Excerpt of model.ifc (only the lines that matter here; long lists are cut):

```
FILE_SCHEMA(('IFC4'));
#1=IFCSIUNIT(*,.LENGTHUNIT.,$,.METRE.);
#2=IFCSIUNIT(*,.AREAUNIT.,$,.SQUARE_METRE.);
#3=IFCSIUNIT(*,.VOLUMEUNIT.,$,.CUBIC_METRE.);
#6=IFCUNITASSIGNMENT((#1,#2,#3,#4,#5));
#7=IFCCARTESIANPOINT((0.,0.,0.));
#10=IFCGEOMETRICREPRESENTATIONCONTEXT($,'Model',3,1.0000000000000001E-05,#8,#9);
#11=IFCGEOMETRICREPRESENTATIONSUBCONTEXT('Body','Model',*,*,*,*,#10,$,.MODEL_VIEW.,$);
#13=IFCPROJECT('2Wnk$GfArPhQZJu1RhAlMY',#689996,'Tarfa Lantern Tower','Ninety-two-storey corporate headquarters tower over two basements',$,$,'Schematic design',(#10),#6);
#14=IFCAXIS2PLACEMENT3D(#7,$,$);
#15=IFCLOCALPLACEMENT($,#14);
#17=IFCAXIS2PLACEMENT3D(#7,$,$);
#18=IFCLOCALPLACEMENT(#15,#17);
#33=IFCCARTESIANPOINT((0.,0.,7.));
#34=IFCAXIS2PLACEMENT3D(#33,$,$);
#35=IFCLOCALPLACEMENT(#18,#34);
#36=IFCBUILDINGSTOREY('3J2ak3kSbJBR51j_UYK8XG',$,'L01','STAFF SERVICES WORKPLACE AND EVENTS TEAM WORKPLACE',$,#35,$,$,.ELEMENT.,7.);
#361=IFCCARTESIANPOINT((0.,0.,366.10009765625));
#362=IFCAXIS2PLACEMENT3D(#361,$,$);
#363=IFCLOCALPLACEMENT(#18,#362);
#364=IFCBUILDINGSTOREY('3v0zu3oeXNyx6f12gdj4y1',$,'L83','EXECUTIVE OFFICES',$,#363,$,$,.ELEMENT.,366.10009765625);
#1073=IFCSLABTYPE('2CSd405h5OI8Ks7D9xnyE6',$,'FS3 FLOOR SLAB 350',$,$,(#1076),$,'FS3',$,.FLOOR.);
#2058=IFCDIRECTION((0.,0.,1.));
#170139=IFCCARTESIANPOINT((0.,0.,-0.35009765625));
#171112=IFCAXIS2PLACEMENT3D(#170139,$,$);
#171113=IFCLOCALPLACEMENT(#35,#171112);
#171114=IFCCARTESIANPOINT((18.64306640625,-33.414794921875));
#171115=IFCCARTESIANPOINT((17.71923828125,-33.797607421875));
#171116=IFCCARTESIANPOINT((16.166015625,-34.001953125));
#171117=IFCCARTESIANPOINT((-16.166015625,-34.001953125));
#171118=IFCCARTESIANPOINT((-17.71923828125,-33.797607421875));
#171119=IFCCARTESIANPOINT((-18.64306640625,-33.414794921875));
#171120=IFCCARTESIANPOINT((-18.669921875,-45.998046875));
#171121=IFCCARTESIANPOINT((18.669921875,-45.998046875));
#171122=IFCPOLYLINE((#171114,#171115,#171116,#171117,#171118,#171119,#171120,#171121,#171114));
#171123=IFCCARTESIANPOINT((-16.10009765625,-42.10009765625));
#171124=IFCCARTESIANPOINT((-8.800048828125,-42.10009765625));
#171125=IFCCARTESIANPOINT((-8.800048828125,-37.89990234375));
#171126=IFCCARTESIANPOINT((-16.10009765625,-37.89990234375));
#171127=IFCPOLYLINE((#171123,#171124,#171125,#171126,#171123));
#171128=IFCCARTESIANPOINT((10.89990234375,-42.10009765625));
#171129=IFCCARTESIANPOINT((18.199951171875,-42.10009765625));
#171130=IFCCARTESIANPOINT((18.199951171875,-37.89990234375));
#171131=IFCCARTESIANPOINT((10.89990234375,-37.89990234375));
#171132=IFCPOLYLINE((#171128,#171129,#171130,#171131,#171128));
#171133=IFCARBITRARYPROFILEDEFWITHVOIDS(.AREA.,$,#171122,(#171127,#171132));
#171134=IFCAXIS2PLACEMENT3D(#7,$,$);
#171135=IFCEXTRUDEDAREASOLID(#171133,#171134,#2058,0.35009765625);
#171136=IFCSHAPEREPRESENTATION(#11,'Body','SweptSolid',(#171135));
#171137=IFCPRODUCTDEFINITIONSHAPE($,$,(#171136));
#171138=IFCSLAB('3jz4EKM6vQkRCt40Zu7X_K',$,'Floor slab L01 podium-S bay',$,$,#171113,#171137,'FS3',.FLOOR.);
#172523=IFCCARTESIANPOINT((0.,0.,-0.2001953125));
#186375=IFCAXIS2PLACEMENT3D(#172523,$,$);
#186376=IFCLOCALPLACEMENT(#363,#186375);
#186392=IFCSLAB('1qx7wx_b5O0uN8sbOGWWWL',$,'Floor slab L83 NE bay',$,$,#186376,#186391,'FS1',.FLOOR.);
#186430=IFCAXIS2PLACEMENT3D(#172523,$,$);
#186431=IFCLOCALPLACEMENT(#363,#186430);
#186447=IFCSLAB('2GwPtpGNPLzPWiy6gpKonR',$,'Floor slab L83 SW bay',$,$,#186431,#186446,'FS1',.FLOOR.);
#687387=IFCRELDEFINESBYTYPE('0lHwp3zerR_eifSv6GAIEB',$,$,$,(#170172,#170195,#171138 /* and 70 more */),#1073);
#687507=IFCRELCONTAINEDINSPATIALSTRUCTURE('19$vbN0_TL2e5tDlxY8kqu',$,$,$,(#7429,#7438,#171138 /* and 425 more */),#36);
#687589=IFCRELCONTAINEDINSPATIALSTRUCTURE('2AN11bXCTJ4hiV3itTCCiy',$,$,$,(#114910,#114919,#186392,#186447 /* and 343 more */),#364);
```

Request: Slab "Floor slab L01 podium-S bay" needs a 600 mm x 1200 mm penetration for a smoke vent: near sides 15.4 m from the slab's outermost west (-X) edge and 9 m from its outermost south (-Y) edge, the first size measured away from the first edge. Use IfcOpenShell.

```python
import numpy as np
import ifcopenshell
import ifcopenshell.api.feature
import ifcopenshell.api.geometry
import ifcopenshell.api.root
import ifcopenshell.geom
import ifcopenshell.util.placement
import ifcopenshell.util.representation
import ifcopenshell.util.shape
import ifcopenshell.util.unit

model = ifcopenshell.open("model.ifc")
unit_scale = ifcopenshell.util.unit.calculate_unit_scale(model)
settings = ifcopenshell.geom.settings()


def volume(element):
    """Net volume in cubic metres, openings subtracted."""
    shape = ifcopenshell.geom.create_shape(settings, element)
    return ifcopenshell.util.shape.get_volume(shape.geometry)


slab = model.by_guid("3jz4EKM6vQkRCt40Zu7X_K")
before = volume(slab)

# Extent in the slab's own axes, in metres. The edges named are its -X and -Y sides.
slab_shape = ifcopenshell.geom.create_shape(settings, slab)
vertices = ifcopenshell.util.shape.get_vertices(slab_shape.geometry)
x_min, y_min, bottom = vertices.min(axis=0)
top = vertices[:, 2].max()

opening = ifcopenshell.api.root.create_entity(model, ifc_class="IfcOpeningElement", name="Smoke vent opening", predefined_type="OPENING")
context = ifcopenshell.util.representation.get_context(model, "Model", "Body", "MODEL_VIEW")
width, depth = 0.6, 1.2
outline = [(0.0, 0.0), (width, 0.0), (width, depth), (0.0, depth), (0.0, 0.0)]
# Overshoot both faces by 50 mm so the cut is clean.
shape = ifcopenshell.api.geometry.add_slab_representation(
    model, context=context, depth=top - bottom + 0.1, polyline=outline
)
ifcopenshell.api.geometry.assign_representation(model, product=opening, representation=shape)

matrix = ifcopenshell.util.placement.get_local_placement(slab.ObjectPlacement)
matrix[:, 3] = matrix @ np.append(np.array([x_min + 15.4, y_min + 9, bottom - 0.05]) / unit_scale, 1.0)
ifcopenshell.api.geometry.edit_object_placement(model, product=opening, matrix=matrix, is_si=False)
ifcopenshell.api.feature.add_feature(model, feature=opening, element=slab)

after = volume(slab)

print(f"slab volume {before:.3f} -> {after:.3f} m3")

model.write("model_edited.ifc")
```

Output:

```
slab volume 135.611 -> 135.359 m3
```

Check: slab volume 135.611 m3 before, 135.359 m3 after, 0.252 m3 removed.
